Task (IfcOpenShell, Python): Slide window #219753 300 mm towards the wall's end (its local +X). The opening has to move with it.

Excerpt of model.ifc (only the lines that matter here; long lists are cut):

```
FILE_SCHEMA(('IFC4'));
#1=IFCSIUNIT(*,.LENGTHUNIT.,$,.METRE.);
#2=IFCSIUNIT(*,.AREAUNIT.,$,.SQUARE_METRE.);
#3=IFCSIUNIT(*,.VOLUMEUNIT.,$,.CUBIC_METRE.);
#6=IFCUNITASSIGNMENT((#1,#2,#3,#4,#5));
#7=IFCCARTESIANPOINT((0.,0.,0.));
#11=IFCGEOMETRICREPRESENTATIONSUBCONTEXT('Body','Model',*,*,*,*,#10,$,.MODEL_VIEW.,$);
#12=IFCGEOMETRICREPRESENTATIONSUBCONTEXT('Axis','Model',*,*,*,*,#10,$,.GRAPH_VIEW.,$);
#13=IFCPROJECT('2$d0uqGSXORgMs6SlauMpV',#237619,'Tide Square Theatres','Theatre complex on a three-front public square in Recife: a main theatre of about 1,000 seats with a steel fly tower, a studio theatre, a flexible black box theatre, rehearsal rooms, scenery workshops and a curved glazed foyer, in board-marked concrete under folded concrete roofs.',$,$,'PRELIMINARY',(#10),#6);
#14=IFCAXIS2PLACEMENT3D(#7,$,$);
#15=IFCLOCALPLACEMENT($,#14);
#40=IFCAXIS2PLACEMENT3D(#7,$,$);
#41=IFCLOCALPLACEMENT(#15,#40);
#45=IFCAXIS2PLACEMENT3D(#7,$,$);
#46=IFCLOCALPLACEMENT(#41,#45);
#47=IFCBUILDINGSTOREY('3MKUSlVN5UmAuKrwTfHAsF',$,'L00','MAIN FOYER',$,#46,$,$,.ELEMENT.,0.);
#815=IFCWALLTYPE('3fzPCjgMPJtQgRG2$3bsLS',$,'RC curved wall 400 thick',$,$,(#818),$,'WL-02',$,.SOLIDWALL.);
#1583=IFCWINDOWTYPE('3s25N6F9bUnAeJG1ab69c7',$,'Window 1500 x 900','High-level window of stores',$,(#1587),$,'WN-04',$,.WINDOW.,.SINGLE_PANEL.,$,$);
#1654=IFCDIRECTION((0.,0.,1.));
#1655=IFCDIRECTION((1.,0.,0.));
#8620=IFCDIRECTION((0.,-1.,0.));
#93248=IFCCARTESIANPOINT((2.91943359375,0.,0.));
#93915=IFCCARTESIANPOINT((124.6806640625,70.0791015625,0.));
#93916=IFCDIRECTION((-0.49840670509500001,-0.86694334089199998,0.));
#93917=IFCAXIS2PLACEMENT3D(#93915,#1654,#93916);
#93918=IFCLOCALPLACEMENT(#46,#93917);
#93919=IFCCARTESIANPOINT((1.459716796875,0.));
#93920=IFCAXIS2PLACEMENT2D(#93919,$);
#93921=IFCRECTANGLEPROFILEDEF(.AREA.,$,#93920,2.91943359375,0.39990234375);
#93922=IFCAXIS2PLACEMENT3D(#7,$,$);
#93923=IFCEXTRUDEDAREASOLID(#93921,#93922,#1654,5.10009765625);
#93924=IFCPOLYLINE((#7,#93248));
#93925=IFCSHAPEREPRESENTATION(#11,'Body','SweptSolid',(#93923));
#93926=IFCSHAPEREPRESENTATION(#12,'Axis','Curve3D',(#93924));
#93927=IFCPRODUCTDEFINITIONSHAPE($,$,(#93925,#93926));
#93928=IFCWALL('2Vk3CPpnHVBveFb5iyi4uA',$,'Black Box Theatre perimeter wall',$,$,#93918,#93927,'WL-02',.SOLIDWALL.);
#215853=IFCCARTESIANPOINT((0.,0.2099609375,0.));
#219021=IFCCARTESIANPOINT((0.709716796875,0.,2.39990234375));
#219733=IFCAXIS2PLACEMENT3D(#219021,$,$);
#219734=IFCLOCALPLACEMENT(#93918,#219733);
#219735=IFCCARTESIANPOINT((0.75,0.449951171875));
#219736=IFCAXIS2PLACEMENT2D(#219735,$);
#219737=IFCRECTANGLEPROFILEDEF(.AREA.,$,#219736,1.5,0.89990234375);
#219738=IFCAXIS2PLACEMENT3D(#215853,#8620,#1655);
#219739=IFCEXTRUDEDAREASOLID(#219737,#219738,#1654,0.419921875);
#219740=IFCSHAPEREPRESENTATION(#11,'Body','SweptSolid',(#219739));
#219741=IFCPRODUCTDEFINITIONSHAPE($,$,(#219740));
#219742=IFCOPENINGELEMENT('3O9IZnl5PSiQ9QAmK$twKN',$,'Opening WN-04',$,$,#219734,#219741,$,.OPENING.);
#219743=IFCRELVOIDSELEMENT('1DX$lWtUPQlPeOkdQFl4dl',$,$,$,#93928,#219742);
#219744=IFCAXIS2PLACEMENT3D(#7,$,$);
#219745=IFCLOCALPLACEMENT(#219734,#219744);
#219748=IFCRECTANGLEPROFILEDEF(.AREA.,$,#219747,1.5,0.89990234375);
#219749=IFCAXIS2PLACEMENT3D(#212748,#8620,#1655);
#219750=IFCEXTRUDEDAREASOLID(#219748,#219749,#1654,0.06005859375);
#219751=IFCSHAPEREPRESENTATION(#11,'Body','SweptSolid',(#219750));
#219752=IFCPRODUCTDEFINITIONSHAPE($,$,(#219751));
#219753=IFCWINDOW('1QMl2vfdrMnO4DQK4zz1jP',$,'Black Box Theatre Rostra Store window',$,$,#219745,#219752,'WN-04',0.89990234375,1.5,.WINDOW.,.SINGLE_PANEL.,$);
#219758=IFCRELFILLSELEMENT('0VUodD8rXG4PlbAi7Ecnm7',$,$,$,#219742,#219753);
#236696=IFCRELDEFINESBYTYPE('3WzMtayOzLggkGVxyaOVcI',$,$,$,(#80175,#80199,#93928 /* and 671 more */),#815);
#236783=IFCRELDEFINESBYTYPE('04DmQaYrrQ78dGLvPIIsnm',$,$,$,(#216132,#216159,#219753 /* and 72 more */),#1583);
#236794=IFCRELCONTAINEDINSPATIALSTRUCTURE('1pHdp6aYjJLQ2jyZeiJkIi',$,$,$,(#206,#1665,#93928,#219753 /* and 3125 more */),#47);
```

```python
import ifcopenshell
import ifcopenshell.api.geometry
import ifcopenshell.util.placement
import ifcopenshell.util.unit

model = ifcopenshell.open("model.ifc")
unit_scale = ifcopenshell.util.unit.calculate_unit_scale(model)

window = model.by_id(219753)
opening = window.FillsVoids[0].RelatingOpeningElement
wall = opening.VoidsElements[0].RelatingBuildingElement

wall_matrix = ifcopenshell.util.placement.get_local_placement(wall.ObjectPlacement)
shift = wall_matrix[:3, 0] * 0.3 / unit_scale
before = ifcopenshell.util.placement.get_local_placement(window.ObjectPlacement)[:3, 3].copy()

# The window is placed relative to its opening, so it follows when the opening moves.
matrix = ifcopenshell.util.placement.get_local_placement(opening.ObjectPlacement)
matrix[:3, 3] += shift
ifcopenshell.api.geometry.edit_object_placement(
    model, product=opening, matrix=matrix, is_si=False, should_transform_children=True
)

after = ifcopenshell.util.placement.get_local_placement(window.ObjectPlacement)[:3, 3]
print("window moved by", (after - before).round(3) + 0.0)

model.write("model_rev.ifc")
```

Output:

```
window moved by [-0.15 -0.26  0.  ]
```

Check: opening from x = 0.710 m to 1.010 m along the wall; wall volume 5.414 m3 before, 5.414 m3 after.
